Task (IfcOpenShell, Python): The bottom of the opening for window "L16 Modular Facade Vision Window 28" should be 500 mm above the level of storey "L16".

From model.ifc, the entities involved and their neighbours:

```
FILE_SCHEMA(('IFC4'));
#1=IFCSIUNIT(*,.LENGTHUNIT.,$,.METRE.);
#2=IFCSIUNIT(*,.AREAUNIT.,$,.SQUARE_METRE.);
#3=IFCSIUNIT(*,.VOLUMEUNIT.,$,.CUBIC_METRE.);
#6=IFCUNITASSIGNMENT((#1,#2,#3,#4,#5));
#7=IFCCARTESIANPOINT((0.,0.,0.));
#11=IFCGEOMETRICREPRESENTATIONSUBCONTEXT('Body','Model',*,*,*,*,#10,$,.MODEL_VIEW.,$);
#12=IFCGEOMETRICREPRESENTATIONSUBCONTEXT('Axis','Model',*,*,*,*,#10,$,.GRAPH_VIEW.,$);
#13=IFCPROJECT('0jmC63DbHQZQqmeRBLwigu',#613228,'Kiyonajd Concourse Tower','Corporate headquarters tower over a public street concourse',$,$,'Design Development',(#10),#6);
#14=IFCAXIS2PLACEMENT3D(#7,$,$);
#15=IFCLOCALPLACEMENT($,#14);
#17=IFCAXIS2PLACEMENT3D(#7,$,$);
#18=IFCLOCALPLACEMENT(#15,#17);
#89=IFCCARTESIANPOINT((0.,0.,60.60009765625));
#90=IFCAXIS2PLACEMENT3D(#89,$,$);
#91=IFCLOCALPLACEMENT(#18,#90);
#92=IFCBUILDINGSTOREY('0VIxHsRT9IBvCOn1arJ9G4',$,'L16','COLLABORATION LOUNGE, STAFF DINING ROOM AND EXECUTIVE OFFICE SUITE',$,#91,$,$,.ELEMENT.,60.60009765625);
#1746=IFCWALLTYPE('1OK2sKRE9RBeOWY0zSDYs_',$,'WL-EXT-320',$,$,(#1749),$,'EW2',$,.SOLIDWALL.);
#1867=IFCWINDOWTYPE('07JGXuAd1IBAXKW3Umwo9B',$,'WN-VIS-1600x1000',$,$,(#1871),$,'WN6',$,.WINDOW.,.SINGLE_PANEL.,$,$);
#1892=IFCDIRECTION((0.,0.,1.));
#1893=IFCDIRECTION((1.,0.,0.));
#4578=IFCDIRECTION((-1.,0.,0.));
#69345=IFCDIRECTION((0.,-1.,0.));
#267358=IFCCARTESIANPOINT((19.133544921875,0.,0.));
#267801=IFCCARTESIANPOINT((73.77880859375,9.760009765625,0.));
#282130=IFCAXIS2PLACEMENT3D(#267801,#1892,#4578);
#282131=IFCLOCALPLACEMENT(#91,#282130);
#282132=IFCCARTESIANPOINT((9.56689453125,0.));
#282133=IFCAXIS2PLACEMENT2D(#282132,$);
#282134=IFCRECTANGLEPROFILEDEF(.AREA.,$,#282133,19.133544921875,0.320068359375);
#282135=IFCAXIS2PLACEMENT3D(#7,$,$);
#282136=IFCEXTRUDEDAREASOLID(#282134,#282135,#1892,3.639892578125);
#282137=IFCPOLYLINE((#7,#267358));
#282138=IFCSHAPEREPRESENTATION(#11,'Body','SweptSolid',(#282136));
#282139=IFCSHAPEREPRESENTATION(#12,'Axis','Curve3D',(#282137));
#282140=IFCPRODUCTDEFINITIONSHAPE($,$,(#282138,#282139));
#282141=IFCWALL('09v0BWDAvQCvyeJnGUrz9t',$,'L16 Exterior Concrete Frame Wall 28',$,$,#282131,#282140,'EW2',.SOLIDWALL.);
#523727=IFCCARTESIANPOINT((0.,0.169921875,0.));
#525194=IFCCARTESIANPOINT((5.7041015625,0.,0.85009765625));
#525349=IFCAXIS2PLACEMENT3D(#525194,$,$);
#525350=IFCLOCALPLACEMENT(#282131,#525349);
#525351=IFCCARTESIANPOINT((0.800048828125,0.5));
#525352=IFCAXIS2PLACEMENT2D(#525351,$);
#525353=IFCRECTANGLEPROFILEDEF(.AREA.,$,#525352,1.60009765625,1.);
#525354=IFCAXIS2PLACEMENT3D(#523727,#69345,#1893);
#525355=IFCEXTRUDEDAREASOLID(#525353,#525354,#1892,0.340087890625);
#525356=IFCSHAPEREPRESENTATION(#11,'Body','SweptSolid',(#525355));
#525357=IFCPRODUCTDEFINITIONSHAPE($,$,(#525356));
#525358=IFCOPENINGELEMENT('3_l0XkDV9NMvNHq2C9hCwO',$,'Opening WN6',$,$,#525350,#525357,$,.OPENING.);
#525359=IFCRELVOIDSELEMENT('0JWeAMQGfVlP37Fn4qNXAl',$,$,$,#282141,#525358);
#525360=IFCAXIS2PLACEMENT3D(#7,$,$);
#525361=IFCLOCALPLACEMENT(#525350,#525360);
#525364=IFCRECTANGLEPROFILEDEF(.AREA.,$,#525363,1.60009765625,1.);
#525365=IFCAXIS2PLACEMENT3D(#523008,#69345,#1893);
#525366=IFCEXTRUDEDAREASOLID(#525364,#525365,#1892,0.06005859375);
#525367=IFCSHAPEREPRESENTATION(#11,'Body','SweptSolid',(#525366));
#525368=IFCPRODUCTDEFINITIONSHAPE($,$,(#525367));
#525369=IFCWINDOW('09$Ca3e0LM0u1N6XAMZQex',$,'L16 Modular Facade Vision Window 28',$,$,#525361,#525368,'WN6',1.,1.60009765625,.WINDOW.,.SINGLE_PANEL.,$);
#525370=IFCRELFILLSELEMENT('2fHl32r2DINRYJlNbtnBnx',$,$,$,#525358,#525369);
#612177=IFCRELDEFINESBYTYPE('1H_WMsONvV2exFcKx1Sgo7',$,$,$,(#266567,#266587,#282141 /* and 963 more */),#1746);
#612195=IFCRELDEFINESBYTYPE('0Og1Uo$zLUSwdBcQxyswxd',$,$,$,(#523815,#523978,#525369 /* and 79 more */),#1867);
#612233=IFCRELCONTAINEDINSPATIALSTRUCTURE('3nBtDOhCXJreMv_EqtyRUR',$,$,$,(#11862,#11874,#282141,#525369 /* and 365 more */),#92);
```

```python
import numpy as np
import ifcopenshell
import ifcopenshell.api.geometry
import ifcopenshell.geom
import ifcopenshell.util.element
import ifcopenshell.util.placement
import ifcopenshell.util.shape
import ifcopenshell.util.unit

model = ifcopenshell.open("model.ifc")
unit_scale = ifcopenshell.util.unit.calculate_unit_scale(model)

window = model.by_id(525369)
opening = window.FillsVoids[0].RelatingOpeningElement
storey = ifcopenshell.util.element.get_container(window, ifc_class="IfcBuildingStorey")
level = ifcopenshell.util.placement.get_local_placement(storey.ObjectPlacement)[2, 3]

# The opening's origin need not be at the sill, so measure its lowest point.
shape = ifcopenshell.geom.create_shape(ifcopenshell.geom.settings(), opening)
bottom = ifcopenshell.util.shape.get_shape_bottom_elevation(shape, shape.geometry) / unit_scale
dz = level + 0.5 - bottom

shift = np.array([0.0, 0.0, dz])
# The window is placed relative to its opening, so it follows when the opening moves.
matrix = ifcopenshell.util.placement.get_local_placement(opening.ObjectPlacement)
matrix[:3, 3] += shift
ifcopenshell.api.geometry.edit_object_placement(
    model, product=opening, matrix=matrix, is_si=False, should_transform_children=True
)

print(f"moved by {dz * unit_scale:+.3f} m")

model.write("model_rev.ifc")
```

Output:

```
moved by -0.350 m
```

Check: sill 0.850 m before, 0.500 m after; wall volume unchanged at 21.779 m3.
